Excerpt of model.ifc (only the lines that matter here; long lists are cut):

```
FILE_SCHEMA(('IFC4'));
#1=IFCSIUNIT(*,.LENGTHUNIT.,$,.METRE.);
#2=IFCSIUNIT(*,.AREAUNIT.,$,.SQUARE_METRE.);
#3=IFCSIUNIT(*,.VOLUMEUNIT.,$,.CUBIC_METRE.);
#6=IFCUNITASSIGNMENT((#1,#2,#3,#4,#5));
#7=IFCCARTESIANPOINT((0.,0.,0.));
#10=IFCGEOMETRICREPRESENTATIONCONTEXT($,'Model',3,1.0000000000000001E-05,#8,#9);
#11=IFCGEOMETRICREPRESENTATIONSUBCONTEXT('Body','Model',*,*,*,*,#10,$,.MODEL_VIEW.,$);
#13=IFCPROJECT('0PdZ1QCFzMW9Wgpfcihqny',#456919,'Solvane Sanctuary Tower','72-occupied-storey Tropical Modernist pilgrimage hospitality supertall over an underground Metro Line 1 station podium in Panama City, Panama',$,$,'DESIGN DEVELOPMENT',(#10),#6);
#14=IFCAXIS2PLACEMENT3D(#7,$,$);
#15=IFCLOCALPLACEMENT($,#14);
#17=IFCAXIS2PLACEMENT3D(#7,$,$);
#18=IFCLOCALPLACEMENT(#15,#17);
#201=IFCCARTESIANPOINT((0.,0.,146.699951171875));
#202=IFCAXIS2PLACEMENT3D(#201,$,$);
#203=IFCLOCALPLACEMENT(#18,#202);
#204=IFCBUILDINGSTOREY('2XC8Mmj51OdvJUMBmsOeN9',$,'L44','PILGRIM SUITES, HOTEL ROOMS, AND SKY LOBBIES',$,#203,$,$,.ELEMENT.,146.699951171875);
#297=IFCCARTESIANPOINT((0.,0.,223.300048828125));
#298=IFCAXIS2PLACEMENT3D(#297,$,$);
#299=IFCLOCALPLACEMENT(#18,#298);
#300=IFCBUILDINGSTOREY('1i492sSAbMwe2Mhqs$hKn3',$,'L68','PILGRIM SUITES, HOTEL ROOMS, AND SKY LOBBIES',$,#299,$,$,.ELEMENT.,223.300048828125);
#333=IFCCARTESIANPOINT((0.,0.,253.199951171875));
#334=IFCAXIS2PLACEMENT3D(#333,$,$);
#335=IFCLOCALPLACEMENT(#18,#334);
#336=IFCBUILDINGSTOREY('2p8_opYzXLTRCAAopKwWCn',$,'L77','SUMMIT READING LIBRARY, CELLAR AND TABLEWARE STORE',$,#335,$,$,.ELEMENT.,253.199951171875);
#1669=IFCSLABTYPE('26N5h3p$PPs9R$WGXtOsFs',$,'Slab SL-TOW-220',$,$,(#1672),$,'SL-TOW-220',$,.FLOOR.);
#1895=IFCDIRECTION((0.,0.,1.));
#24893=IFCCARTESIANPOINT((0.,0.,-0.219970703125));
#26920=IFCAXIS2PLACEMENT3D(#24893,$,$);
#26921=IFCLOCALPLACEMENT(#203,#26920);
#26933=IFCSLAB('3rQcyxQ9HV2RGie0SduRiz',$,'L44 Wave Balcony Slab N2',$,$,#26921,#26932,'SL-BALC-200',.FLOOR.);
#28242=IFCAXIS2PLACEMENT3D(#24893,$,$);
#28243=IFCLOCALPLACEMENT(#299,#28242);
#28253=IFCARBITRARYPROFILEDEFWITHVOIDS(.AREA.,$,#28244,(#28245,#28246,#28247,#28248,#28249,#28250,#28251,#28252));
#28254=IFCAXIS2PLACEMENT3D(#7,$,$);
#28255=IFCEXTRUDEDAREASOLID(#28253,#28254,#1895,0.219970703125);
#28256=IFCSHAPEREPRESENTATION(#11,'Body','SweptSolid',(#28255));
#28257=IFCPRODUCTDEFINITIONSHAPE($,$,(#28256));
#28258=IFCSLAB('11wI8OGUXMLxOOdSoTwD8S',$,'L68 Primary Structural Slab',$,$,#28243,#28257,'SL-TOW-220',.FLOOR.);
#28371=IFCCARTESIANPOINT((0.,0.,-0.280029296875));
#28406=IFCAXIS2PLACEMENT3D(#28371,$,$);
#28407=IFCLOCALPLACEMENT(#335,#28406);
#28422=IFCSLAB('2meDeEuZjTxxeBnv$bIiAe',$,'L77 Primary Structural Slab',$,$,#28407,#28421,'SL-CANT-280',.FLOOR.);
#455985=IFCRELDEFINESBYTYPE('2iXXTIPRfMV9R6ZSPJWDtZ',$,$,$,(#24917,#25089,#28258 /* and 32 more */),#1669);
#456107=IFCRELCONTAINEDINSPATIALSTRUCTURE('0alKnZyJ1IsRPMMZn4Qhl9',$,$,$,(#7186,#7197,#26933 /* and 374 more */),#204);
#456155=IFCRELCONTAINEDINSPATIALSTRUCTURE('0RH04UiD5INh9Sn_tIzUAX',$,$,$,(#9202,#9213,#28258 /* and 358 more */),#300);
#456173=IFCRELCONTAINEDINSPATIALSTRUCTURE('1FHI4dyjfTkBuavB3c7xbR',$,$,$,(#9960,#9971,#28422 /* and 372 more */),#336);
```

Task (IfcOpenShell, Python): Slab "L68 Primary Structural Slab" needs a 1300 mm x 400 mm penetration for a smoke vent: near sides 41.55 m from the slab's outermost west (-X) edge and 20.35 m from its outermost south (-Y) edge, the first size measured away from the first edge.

```python
import numpy as np
import ifcopenshell
import ifcopenshell.api.feature
import ifcopenshell.api.geometry
import ifcopenshell.api.root
import ifcopenshell.geom
import ifcopenshell.util.placement
import ifcopenshell.util.representation
import ifcopenshell.util.shape
import ifcopenshell.util.unit

model = ifcopenshell.open("model.ifc")
unit_scale = ifcopenshell.util.unit.calculate_unit_scale(model)
settings = ifcopenshell.geom.settings()


def volume(element):
    """Net volume in cubic metres, openings subtracted."""
    shape = ifcopenshell.geom.create_shape(settings, element)
    return ifcopenshell.util.shape.get_volume(shape.geometry)


slab = model.by_id(28258)
before = volume(slab)

# Extent in the slab's own axes, in metres. The edges named are its -X and -Y sides.
slab_shape = ifcopenshell.geom.create_shape(settings, slab)
vertices = ifcopenshell.util.shape.get_vertices(slab_shape.geometry)
x_min, y_min, bottom = vertices.min(axis=0)
top = vertices[:, 2].max()

opening = ifcopenshell.api.root.create_entity(model, ifc_class="IfcOpeningElement", name="Smoke vent opening", predefined_type="OPENING")
context = ifcopenshell.util.representation.get_context(model, "Model", "Body", "MODEL_VIEW")
width, depth = 1.3, 0.4
outline = [(0.0, 0.0), (width, 0.0), (width, depth), (0.0, depth), (0.0, 0.0)]
# Overshoot both faces by 50 mm so the cut is clean.
shape = ifcopenshell.api.geometry.add_slab_representation(
    model, context=context, depth=top - bottom + 0.1, polyline=outline
)
ifcopenshell.api.geometry.assign_representation(model, product=opening, representation=shape)

matrix = ifcopenshell.util.placement.get_local_placement(slab.ObjectPlacement)
matrix[:, 3] = matrix @ np.append(np.array([x_min + 41.55, y_min + 20.35, bottom - 0.05]) / unit_scale, 1.0)
ifcopenshell.api.geometry.edit_object_placement(model, product=opening, matrix=matrix, is_si=False)
ifcopenshell.api.feature.add_feature(model, feature=opening, element=slab)

after = volume(slab)

print(f"slab volume {before:.3f} -> {after:.3f} m3")

model.write("model_updated.ifc")
```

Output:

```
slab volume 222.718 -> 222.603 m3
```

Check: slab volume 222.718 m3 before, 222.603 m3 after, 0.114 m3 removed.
